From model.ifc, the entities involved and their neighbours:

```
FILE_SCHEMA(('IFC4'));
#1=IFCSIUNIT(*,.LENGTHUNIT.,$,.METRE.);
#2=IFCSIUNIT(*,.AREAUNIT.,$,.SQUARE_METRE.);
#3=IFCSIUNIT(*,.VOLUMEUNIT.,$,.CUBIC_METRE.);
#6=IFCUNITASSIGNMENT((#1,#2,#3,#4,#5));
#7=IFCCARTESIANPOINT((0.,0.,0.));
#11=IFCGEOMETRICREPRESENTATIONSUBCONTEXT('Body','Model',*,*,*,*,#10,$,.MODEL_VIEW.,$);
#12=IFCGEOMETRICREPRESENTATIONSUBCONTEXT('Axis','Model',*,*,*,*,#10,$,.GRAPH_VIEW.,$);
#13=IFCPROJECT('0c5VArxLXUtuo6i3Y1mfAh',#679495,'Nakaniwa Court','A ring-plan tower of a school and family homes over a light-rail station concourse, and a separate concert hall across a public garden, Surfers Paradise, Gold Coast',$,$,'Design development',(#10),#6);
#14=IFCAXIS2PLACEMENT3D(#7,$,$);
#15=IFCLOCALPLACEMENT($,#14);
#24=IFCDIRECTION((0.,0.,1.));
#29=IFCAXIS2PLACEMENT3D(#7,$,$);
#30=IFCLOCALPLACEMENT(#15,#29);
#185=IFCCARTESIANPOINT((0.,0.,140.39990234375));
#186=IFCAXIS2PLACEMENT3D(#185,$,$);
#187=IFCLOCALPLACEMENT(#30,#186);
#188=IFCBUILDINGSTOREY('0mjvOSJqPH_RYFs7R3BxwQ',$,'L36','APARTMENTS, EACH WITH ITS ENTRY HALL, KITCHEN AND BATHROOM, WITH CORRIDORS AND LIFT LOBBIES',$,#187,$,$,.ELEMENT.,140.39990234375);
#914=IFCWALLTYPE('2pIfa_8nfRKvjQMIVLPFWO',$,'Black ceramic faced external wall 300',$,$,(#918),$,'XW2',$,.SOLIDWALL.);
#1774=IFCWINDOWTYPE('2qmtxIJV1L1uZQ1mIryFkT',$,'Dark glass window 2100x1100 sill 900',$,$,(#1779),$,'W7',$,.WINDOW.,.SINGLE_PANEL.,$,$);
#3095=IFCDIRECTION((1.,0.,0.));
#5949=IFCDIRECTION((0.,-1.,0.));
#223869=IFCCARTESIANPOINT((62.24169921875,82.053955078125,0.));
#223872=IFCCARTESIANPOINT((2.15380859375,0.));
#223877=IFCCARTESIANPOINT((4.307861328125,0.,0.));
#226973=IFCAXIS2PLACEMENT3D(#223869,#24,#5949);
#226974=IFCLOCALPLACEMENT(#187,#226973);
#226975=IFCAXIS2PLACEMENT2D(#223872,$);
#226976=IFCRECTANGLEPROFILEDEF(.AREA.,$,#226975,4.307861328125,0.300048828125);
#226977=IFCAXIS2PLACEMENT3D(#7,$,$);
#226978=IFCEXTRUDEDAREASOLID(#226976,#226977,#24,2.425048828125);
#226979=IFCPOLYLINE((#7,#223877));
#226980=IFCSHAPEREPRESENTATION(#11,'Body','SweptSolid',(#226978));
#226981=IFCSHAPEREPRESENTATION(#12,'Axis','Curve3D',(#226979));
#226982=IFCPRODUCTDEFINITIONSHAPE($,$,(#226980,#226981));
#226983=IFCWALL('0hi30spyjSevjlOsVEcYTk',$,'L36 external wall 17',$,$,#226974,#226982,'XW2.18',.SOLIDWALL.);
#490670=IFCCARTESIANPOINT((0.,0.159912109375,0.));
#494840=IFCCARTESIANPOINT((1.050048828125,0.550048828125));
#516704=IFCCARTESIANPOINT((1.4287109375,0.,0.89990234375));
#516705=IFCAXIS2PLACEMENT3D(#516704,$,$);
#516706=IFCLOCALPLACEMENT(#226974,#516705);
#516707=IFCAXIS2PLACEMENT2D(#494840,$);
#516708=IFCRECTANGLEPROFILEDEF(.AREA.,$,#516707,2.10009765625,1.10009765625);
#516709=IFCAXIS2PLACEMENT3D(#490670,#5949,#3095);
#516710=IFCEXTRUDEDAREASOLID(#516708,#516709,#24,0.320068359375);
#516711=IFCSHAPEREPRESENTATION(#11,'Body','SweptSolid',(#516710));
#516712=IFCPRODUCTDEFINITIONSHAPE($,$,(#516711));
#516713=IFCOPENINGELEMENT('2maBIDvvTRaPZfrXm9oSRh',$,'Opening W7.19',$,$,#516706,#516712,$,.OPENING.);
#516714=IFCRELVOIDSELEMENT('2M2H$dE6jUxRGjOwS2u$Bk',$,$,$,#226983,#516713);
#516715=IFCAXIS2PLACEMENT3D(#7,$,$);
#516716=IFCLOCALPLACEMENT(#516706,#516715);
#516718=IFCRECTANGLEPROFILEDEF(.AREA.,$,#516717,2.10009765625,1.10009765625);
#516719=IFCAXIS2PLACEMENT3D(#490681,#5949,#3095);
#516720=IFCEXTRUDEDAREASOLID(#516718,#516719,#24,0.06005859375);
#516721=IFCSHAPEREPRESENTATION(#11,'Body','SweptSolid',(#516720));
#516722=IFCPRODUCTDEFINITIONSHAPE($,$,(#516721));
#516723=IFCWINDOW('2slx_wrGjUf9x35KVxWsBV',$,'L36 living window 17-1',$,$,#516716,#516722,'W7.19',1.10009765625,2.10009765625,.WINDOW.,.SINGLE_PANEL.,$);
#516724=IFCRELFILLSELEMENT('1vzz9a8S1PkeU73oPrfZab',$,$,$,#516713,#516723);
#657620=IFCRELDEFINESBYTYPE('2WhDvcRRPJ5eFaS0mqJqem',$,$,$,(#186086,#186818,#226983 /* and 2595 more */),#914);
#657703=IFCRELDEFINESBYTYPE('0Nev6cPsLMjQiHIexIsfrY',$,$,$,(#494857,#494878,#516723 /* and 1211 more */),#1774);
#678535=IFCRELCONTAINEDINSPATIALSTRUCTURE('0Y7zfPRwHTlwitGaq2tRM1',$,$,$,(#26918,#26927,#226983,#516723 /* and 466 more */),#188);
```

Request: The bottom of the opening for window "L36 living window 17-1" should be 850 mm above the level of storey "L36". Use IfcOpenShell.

```python
import numpy as np
import ifcopenshell
import ifcopenshell.api.geometry
import ifcopenshell.geom
import ifcopenshell.util.element
import ifcopenshell.util.placement
import ifcopenshell.util.shape
import ifcopenshell.util.unit

model = ifcopenshell.open("model.ifc")
unit_scale = ifcopenshell.util.unit.calculate_unit_scale(model)

window = model.by_guid("2slx_wrGjUf9x35KVxWsBV")
opening = window.FillsVoids[0].RelatingOpeningElement
storey = ifcopenshell.util.element.get_container(window, ifc_class="IfcBuildingStorey")
level = ifcopenshell.util.placement.get_local_placement(storey.ObjectPlacement)[2, 3]

# The opening's origin need not be at the sill, so measure its lowest point.
shape = ifcopenshell.geom.create_shape(ifcopenshell.geom.settings(), opening)
bottom = ifcopenshell.util.shape.get_shape_bottom_elevation(shape, shape.geometry) / unit_scale
dz = level + 0.85 / unit_scale - bottom

shift = np.array([0.0, 0.0, dz])
# The window is placed relative to its opening, so it follows when the opening moves.
matrix = ifcopenshell.util.placement.get_local_placement(opening.ObjectPlacement)
matrix[:3, 3] += shift
ifcopenshell.api.geometry.edit_object_placement(
    model, product=opening, matrix=matrix, is_si=False, should_transform_children=True
)

print(f"moved by {dz * unit_scale:+.3f} m")

model.write("model_edited.ifc")
```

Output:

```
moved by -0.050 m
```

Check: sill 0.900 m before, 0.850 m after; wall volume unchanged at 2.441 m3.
